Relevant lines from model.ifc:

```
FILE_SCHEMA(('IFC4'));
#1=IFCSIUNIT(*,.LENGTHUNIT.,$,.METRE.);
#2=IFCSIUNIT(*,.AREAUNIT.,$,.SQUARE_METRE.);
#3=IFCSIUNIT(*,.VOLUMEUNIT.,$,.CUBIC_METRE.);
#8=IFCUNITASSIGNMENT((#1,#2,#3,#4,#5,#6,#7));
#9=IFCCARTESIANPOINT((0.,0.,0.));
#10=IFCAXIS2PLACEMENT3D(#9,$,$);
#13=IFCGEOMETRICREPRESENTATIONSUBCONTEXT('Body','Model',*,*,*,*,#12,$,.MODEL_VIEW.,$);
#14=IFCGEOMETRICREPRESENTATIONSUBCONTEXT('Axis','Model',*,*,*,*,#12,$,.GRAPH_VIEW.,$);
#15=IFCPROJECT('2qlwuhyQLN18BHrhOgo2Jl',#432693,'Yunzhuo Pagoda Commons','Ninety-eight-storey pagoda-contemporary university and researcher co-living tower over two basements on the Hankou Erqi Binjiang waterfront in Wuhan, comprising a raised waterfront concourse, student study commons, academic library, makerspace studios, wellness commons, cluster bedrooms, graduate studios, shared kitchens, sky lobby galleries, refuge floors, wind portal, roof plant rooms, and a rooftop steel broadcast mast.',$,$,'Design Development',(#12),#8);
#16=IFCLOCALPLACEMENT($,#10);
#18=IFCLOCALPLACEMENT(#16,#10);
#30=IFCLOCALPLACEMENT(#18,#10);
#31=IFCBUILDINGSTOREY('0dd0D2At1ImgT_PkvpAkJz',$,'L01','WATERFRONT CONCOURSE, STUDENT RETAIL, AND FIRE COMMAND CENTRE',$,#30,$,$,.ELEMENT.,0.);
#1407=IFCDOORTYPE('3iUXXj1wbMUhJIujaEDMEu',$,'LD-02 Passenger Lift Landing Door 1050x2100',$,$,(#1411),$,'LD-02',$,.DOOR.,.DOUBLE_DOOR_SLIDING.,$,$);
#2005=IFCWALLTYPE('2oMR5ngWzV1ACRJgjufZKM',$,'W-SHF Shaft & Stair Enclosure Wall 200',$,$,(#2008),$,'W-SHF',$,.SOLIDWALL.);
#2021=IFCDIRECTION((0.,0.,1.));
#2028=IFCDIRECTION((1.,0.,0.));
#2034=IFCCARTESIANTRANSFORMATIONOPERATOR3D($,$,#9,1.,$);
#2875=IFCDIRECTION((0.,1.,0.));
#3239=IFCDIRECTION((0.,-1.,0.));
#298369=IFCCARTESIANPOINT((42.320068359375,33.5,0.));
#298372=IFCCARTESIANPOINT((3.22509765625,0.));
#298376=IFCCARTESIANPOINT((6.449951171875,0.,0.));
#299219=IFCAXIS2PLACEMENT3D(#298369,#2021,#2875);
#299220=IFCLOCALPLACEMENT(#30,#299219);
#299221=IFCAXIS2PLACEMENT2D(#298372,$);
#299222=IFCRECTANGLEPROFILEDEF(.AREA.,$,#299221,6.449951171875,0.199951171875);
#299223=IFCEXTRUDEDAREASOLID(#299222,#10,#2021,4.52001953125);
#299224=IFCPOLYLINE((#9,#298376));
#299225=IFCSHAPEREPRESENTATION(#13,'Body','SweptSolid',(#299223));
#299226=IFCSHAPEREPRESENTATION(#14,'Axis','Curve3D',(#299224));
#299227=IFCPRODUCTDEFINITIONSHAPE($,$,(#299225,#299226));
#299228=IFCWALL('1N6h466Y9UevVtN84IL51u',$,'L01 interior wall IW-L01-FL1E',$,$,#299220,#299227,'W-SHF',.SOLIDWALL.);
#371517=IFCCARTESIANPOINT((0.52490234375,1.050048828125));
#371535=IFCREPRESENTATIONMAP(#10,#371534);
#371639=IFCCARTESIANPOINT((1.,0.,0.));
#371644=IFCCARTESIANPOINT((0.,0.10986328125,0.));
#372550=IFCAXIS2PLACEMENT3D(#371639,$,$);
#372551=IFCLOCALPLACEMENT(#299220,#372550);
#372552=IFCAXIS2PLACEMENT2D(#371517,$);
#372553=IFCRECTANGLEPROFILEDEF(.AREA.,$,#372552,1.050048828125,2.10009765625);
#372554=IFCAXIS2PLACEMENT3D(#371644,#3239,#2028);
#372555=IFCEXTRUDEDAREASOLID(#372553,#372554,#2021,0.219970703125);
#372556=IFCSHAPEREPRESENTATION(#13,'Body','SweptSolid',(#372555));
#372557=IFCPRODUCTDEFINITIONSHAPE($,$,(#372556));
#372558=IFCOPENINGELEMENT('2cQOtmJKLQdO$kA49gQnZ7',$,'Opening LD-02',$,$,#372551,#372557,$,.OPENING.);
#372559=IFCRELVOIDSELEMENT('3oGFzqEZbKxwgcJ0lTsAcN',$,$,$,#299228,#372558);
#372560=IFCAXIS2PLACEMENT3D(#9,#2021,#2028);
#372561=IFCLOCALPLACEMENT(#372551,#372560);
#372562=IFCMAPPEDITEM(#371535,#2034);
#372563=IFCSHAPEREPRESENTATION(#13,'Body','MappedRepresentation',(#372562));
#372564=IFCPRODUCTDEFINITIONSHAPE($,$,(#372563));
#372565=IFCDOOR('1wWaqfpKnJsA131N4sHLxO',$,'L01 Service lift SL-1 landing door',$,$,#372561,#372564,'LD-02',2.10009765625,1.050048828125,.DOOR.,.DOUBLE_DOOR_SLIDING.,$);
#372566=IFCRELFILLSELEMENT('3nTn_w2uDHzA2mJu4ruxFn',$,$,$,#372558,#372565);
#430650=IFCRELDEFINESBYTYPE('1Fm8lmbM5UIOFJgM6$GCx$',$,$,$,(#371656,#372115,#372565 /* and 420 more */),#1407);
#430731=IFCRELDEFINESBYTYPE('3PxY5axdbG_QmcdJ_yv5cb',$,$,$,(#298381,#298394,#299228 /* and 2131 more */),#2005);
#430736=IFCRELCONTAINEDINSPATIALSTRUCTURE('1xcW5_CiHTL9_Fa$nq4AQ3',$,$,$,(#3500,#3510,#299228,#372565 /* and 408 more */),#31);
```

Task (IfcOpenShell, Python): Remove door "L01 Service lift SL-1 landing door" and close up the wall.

```python
import ifcopenshell
import ifcopenshell.api.feature
import ifcopenshell.api.root
import ifcopenshell.geom
import ifcopenshell.util.shape

model = ifcopenshell.open("model.ifc")
settings = ifcopenshell.geom.settings()


def volume(element):
    """Net volume in cubic metres, openings subtracted."""
    shape = ifcopenshell.geom.create_shape(settings, element)
    return ifcopenshell.util.shape.get_volume(shape.geometry)


door = model.by_id(372565)
opening = door.FillsVoids[0].RelatingOpeningElement
wall = opening.VoidsElements[0].RelatingBuildingElement
before = volume(wall)

ifcopenshell.api.root.remove_product(model, product=door)
ifcopenshell.api.feature.remove_feature(model, feature=opening)

after = volume(wall)

print(f"wall volume {before:.3f} -> {after:.3f} m3")

model.write("model_rev.ifc")
```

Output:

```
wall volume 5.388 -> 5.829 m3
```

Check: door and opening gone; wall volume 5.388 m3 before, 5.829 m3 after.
